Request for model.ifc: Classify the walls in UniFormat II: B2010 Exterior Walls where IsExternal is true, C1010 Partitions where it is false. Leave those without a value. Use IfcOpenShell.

First a look at what the model holds.

```python
import ifcopenshell
import ifcopenshell.util.element

model = ifcopenshell.open("model.ifc")
print(model.schema)
print("classifications:", [c.Name for c in model.by_type("IfcClassification")])
values = [ifcopenshell.util.element.get_pset(e, "Pset_WallCommon", "IsExternal") for e in model.by_type("IfcWall")]
for value in (True, False, None):
    print("IsExternal", value, values.count(value))
```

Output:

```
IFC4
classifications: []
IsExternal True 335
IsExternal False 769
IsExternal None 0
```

```python
import ifcopenshell
import ifcopenshell.api.classification
import ifcopenshell.util.element

model = ifcopenshell.open("model.ifc")

system = ifcopenshell.api.classification.add_classification(model, classification="UniFormat II")

walls = model.by_type("IfcWall")
external = {e: ifcopenshell.util.element.get_pset(e, "Pset_WallCommon", "IsExternal") for e in walls}
for flag, code, name in ((True, "B2010", "Exterior Walls"), (False, "C1010", "Partitions")):
    products = [e for e in walls if external[e] is flag]
    ifcopenshell.api.classification.add_reference(
        model, products=products, classification=system, identification=code, name=name
    )
    print(code, len(products))

model.write("model_updated.ifc")
```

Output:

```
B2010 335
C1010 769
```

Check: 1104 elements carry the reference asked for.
